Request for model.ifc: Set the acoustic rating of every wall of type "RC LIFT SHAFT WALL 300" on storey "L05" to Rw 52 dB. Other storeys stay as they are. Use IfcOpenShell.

First a look at what the model holds.

```python
import ifcopenshell
import ifcopenshell.util.element

model = ifcopenshell.open("model.ifc")
print(model.schema)
storey = next(s for s in model.by_type("IfcBuildingStorey") if s.Name == "L05")
walls = [e for e in ifcopenshell.util.element.get_decomposition(storey) if e.is_a("IfcWall")]
seen = {}
for e in walls:
    element_type = ifcopenshell.util.element.get_type(e)
    key = (element_type.Name if element_type != e and element_type else None, ifcopenshell.util.element.get_pset(e, "Pset_WallCommon", "AcousticRating"))
    seen[key] = seen.get(key, 0) + 1
for (name, value), count in sorted(seen.items(), key=str):
    print(count, "x", name, "|", value)
```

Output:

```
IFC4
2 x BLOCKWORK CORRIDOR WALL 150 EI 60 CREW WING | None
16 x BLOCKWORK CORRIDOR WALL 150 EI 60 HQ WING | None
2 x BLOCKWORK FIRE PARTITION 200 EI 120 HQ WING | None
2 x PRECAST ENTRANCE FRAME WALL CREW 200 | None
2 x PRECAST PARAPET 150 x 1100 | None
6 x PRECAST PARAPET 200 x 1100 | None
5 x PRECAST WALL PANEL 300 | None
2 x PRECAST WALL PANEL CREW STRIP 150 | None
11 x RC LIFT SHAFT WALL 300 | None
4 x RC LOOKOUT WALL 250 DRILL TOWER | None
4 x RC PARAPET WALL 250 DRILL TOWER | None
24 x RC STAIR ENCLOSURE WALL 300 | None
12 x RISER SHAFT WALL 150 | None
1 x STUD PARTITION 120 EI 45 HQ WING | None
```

```python
import ifcopenshell
import ifcopenshell.api.pset
import ifcopenshell.util.element

model = ifcopenshell.open("model.ifc")

storey = next(s for s in model.by_type("IfcBuildingStorey") if s.Name == "L05")
walls = [e for e in ifcopenshell.util.element.get_decomposition(storey) if e.is_a("IfcWall")]

count = 0
for e in walls:
    element_type = ifcopenshell.util.element.get_type(e)
    if element_type in (None, e) or element_type.Name != "RC LIFT SHAFT WALL 300":
        continue
    # add_pset returns the element's existing set when there is one.
    pset = ifcopenshell.api.pset.add_pset(model, product=e, name="Pset_WallCommon")
    ifcopenshell.api.pset.edit_pset(model, pset=pset, properties={"AcousticRating": "Rw 52 dB"})
    count += 1

print(count, "walls updated")

model.write("model_v2.ifc")
```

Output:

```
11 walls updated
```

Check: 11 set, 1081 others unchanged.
